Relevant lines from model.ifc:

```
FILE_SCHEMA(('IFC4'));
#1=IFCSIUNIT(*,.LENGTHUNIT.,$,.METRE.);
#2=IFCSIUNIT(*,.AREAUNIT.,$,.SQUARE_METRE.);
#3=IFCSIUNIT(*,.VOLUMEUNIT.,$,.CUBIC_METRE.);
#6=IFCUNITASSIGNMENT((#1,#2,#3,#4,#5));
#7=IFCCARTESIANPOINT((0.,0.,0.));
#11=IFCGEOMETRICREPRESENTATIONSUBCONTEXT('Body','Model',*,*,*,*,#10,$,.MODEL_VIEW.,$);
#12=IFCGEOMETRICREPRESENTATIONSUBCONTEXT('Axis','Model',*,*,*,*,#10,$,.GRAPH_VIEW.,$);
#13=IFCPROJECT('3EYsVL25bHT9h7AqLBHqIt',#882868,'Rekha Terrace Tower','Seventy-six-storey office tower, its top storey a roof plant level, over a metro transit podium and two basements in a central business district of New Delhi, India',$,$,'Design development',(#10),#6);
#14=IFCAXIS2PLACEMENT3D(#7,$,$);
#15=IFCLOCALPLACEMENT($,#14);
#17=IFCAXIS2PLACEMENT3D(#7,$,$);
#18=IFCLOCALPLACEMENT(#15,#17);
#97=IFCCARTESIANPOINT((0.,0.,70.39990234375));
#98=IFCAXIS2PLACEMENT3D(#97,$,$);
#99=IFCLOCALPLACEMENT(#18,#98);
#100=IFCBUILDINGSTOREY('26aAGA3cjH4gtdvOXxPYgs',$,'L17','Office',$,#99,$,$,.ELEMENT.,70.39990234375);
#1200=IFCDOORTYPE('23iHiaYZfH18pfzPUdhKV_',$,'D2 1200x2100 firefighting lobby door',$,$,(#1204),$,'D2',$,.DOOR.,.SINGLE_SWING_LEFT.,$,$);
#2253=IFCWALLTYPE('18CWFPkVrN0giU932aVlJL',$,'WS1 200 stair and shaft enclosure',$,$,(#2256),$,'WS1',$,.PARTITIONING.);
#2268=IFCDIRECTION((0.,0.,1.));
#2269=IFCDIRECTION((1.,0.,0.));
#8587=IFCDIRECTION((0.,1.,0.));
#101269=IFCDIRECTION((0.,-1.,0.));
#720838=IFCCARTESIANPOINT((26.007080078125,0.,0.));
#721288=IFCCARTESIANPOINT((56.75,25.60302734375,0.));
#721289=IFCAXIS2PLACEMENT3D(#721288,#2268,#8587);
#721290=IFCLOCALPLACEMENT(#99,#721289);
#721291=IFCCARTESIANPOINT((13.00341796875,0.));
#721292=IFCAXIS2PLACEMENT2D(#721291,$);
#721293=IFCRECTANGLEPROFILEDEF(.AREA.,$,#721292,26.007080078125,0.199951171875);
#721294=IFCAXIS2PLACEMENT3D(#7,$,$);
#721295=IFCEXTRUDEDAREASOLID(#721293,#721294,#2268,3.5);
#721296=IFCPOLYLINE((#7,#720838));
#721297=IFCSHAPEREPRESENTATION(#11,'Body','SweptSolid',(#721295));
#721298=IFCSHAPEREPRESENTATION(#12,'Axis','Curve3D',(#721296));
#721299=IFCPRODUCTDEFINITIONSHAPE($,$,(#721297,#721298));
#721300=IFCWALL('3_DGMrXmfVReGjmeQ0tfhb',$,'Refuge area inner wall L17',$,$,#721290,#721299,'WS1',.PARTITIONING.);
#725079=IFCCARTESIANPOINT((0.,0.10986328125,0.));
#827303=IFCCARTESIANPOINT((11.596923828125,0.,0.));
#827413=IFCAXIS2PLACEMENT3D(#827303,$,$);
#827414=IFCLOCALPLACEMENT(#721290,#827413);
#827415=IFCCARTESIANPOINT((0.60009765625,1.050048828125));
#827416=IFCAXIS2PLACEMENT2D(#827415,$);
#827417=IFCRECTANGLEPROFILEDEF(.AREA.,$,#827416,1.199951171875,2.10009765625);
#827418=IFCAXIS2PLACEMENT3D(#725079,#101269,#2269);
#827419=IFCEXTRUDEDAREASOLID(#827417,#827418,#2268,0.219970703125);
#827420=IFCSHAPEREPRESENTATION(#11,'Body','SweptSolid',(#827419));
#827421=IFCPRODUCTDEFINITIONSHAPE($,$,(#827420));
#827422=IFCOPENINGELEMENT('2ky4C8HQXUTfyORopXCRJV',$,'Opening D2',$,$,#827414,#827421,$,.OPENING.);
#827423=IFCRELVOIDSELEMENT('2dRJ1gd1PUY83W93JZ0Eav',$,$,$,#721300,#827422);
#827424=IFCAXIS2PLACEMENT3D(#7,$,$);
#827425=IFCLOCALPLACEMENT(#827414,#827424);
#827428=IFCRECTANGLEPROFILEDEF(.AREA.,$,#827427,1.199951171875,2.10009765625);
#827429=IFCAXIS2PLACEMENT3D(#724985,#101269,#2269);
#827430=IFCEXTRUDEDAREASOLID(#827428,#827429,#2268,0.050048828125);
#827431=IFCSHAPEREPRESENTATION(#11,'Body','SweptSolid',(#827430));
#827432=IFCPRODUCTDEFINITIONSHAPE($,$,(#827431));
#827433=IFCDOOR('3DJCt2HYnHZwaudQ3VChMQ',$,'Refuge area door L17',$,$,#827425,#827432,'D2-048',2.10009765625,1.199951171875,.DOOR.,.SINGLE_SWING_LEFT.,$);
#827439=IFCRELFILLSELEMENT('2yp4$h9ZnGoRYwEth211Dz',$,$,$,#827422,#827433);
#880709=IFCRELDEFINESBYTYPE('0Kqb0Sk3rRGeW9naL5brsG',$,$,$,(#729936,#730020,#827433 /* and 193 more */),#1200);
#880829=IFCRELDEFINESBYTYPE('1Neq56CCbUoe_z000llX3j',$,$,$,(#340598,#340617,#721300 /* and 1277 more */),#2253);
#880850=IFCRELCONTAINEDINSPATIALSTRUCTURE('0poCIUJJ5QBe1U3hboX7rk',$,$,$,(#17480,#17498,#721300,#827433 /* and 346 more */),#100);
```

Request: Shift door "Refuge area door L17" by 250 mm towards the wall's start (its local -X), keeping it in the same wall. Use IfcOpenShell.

```python
import ifcopenshell
import ifcopenshell.api.geometry
import ifcopenshell.util.placement

model = ifcopenshell.open("model.ifc")

door = model.by_guid("3DJCt2HYnHZwaudQ3VChMQ")
opening = door.FillsVoids[0].RelatingOpeningElement
wall = opening.VoidsElements[0].RelatingBuildingElement

wall_matrix = ifcopenshell.util.placement.get_local_placement(wall.ObjectPlacement)
shift = wall_matrix[:3, 0] * -0.25
before = ifcopenshell.util.placement.get_local_placement(door.ObjectPlacement)[:3, 3].copy()

# The door is placed relative to its opening, so it follows when the opening moves.
matrix = ifcopenshell.util.placement.get_local_placement(opening.ObjectPlacement)
matrix[:3, 3] += shift
ifcopenshell.api.geometry.edit_object_placement(
    model, product=opening, matrix=matrix, is_si=False, should_transform_children=True
)

after = ifcopenshell.util.placement.get_local_placement(door.ObjectPlacement)[:3, 3]
print("door moved by", (after - before).round(3) + 0.0)

model.write("model_rev.ifc")
```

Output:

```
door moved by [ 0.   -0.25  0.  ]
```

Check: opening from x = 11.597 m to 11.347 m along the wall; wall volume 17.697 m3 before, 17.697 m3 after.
